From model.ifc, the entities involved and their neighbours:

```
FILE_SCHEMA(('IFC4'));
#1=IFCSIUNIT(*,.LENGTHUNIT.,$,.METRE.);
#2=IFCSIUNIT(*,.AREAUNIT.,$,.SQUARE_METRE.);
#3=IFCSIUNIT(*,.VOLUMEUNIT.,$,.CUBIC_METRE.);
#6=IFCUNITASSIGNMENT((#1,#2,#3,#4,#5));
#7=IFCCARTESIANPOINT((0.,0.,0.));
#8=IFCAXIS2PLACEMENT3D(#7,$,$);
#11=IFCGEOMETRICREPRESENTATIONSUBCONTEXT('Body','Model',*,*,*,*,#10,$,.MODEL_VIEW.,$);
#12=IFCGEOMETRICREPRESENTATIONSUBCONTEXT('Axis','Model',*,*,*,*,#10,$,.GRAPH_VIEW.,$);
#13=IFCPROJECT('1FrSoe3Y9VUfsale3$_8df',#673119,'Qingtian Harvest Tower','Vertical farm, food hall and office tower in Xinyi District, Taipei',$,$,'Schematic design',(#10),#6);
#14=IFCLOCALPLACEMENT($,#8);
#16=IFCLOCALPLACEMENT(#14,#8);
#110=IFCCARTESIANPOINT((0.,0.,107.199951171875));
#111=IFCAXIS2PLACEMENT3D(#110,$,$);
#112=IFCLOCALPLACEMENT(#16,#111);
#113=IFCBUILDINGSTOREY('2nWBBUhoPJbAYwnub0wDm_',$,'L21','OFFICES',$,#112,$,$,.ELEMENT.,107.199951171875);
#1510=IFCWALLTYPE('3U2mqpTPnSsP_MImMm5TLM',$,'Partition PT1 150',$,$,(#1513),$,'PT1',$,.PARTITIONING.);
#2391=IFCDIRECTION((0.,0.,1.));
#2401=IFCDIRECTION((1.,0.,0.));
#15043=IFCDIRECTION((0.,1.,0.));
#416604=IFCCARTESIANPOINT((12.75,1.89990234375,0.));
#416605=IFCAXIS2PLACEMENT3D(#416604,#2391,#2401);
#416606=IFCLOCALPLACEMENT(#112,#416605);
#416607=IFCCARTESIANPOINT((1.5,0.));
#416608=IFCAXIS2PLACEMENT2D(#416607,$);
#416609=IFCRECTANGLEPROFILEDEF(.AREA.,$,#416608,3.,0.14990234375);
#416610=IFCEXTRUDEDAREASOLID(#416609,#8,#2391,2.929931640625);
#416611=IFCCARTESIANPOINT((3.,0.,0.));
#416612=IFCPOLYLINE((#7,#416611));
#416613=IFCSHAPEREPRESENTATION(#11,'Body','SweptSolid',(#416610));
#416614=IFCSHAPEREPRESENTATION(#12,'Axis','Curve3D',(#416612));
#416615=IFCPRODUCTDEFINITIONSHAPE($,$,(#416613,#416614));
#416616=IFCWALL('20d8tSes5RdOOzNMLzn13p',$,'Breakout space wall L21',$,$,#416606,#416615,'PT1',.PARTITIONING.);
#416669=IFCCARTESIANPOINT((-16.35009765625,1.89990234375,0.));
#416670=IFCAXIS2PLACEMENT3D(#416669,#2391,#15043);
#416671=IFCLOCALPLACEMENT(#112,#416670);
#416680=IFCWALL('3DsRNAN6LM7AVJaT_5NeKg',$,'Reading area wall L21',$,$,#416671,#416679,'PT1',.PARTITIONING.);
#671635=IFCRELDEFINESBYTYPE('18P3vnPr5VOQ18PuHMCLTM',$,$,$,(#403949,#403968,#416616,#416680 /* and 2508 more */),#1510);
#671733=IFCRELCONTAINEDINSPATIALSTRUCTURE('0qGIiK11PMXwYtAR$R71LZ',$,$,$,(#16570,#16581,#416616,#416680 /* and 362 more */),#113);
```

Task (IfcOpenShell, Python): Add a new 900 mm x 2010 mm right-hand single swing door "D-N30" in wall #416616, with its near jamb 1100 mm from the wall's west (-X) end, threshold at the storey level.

```python
import numpy as np
import ifcopenshell
import ifcopenshell.api.feature
import ifcopenshell.api.geometry
import ifcopenshell.api.root
import ifcopenshell.api.spatial
import ifcopenshell.geom
import ifcopenshell.util.element
import ifcopenshell.util.placement
import ifcopenshell.util.representation
import ifcopenshell.util.shape
import ifcopenshell.util.unit

model = ifcopenshell.open("model.ifc")
unit_scale = ifcopenshell.util.unit.calculate_unit_scale(model)
settings = ifcopenshell.geom.settings()


def volume(element):
    """Net volume in cubic metres, openings subtracted."""
    shape = ifcopenshell.geom.create_shape(settings, element)
    return ifcopenshell.util.shape.get_volume(shape.geometry)


wall = model.by_guid("20d8tSes5RdOOzNMLzn13p")
storey = ifcopenshell.util.element.get_container(wall, ifc_class="IfcBuildingStorey")
context = ifcopenshell.util.representation.get_context(model, "Model", "Body", "MODEL_VIEW")
before = volume(wall)

width, height, from_end, sill = 0.9, 2.01, 1.1, 0.0  # metres

# The wall runs along its own X axis, and the end named is its -X end.
wall_shape = ifcopenshell.geom.create_shape(settings, wall)
x, y, z = ifcopenshell.util.shape.get_vertices(wall_shape.geometry).T
start = x.min() + from_end
face, thickness = float(y.min()), float(y.max() - y.min())
wall_matrix = ifcopenshell.util.placement.get_local_placement(wall.ObjectPlacement)
level = ifcopenshell.util.placement.get_local_placement(storey.ObjectPlacement)[2, 3]


def in_wall(x, y):
    """Placement at x, y metres in the wall's axes, at sill height."""
    matrix = wall_matrix.copy()
    matrix[:, 3] = wall_matrix @ np.array([x / unit_scale, y / unit_scale, 0.0, 1.0])
    matrix[2, 3] = level + sill / unit_scale
    return matrix


# Opening: a box that overshoots both wall faces by 50 mm.
opening = ifcopenshell.api.root.create_entity(model, ifc_class="IfcOpeningElement", predefined_type="OPENING")
box = ifcopenshell.api.geometry.add_wall_representation(
    model, context=context, length=width, height=height, thickness=thickness + 0.1
)
ifcopenshell.api.geometry.assign_representation(model, product=opening, representation=box)
ifcopenshell.api.geometry.edit_object_placement(model, product=opening, matrix=in_wall(start, face - 0.05), is_si=False)
ifcopenshell.api.feature.add_feature(model, feature=opening, element=wall)

door = ifcopenshell.api.root.create_entity(model, ifc_class="IfcDoor", name="D-N30", predefined_type="DOOR")
door.OverallWidth, door.OverallHeight = width / unit_scale, height / unit_scale
door.OperationType = "SINGLE_SWING_RIGHT"
body = ifcopenshell.api.geometry.add_door_representation(
    model,
    context=context,
    overall_width=door.OverallWidth,
    overall_height=door.OverallHeight,
    operation_type="SINGLE_SWING_RIGHT",
    lining_properties={"LiningDepth": thickness / unit_scale, "ThresholdDepth": thickness / unit_scale},
)
ifcopenshell.api.geometry.assign_representation(model, product=door, representation=body)
ifcopenshell.api.spatial.assign_container(model, products=[door], relating_structure=storey)
ifcopenshell.api.feature.add_filling(model, opening=opening, element=door)

# The lining spans the wall, so the door starts at the wall face.
ifcopenshell.api.geometry.edit_object_placement(model, product=door, matrix=in_wall(start, face), is_si=False)

after = volume(wall)

print(f"wall volume {before:.3f} -> {after:.3f} m3")

model.write("model_rev.ifc")
```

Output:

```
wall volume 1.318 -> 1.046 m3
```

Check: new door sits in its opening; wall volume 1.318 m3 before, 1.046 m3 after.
